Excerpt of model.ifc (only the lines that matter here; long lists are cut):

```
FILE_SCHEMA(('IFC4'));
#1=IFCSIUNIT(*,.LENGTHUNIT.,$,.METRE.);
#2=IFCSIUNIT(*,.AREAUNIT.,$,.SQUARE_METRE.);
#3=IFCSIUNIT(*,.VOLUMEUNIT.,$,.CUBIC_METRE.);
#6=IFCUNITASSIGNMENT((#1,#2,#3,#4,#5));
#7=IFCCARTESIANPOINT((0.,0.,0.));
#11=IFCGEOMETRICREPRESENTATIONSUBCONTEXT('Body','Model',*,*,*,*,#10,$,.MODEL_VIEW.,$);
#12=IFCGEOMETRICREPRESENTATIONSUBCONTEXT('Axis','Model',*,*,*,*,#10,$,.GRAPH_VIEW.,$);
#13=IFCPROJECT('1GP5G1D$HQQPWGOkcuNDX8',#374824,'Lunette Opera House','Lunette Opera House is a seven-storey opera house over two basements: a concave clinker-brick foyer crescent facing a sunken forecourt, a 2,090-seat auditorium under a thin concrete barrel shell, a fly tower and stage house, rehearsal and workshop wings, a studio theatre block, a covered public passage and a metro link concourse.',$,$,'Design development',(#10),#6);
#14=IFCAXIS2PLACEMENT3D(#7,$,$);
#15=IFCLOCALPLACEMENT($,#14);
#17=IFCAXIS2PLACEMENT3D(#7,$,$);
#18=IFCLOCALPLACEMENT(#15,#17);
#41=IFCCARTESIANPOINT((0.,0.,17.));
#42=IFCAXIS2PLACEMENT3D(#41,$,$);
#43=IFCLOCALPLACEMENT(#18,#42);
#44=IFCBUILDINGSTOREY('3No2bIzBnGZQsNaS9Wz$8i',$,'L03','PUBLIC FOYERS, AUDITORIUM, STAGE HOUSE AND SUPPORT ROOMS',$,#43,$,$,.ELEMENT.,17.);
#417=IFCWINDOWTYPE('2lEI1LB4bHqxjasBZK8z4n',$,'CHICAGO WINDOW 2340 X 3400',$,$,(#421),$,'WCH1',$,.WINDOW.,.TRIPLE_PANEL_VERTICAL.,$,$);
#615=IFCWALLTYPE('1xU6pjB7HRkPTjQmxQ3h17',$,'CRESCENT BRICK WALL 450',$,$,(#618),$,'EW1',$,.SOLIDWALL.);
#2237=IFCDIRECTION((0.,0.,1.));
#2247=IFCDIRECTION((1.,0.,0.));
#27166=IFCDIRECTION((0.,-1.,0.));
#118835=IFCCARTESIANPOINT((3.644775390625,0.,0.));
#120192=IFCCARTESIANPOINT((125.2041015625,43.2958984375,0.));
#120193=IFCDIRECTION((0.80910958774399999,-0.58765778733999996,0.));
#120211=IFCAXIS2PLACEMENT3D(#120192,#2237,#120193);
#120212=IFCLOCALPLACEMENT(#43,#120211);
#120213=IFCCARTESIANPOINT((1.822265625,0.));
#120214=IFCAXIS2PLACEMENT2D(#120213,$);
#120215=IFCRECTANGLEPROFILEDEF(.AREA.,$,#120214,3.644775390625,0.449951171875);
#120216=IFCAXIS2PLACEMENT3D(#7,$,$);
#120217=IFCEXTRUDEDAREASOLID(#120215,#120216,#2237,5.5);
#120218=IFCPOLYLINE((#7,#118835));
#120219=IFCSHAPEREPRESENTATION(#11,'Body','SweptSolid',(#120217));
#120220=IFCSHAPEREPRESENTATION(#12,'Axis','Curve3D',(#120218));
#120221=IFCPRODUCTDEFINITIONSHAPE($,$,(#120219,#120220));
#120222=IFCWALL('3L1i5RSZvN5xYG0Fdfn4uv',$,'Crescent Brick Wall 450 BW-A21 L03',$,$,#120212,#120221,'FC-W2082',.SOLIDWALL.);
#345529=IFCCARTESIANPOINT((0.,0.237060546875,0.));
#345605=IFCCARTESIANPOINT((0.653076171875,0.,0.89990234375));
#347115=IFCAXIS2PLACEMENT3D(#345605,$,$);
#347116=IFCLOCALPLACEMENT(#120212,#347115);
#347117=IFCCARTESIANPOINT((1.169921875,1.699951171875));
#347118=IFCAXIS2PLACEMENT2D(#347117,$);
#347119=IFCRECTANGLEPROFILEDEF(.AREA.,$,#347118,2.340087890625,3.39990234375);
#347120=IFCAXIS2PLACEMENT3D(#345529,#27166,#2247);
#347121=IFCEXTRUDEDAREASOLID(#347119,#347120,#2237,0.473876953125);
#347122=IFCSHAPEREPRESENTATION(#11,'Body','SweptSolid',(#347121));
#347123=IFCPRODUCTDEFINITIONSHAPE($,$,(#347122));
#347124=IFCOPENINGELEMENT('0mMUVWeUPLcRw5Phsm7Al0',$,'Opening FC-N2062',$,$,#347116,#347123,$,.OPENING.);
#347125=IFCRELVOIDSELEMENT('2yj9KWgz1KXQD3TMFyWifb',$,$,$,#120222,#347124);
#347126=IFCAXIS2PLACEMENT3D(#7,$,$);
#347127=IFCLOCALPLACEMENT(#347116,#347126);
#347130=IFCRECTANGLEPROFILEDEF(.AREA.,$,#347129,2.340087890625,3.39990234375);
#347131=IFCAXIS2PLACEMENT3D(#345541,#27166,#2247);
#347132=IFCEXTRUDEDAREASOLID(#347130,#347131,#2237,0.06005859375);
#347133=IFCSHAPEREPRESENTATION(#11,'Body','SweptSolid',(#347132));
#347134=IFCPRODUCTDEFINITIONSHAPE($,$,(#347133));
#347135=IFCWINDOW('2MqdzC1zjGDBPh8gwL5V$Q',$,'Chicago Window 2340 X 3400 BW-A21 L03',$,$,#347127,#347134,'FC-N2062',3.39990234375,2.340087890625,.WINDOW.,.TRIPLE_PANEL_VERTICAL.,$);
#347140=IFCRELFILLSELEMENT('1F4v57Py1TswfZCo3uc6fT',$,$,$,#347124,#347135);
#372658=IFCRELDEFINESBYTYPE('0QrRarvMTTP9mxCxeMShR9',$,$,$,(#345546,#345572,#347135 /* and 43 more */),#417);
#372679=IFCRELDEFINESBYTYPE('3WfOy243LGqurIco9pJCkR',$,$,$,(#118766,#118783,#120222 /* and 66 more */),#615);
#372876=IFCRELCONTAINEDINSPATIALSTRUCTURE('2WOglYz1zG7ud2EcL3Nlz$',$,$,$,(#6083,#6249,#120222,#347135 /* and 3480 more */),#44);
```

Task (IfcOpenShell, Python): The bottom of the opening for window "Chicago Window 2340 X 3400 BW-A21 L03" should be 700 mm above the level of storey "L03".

```python
import numpy as np
import ifcopenshell
import ifcopenshell.api.geometry
import ifcopenshell.geom
import ifcopenshell.util.element
import ifcopenshell.util.placement
import ifcopenshell.util.shape
import ifcopenshell.util.unit

model = ifcopenshell.open("model.ifc")
unit_scale = ifcopenshell.util.unit.calculate_unit_scale(model)

window = model.by_guid("2MqdzC1zjGDBPh8gwL5V$Q")
opening = window.FillsVoids[0].RelatingOpeningElement
storey = ifcopenshell.util.element.get_container(window, ifc_class="IfcBuildingStorey")
level = ifcopenshell.util.placement.get_local_placement(storey.ObjectPlacement)[2, 3]

# The opening's origin need not be at the sill, so measure its lowest point.
shape = ifcopenshell.geom.create_shape(ifcopenshell.geom.settings(), opening)
bottom = ifcopenshell.util.shape.get_shape_bottom_elevation(shape, shape.geometry) / unit_scale
dz = level + 0.7 / unit_scale - bottom

shift = np.array([0.0, 0.0, dz])
# The window is placed relative to its opening, so it follows when the opening moves.
matrix = ifcopenshell.util.placement.get_local_placement(opening.ObjectPlacement)
matrix[:3, 3] += shift
ifcopenshell.api.geometry.edit_object_placement(
    model, product=opening, matrix=matrix, is_si=False, should_transform_children=True
)

print(f"moved by {dz * unit_scale:+.3f} m")

model.write("model_v2.ifc")
```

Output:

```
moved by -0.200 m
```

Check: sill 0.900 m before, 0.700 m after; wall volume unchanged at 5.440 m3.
